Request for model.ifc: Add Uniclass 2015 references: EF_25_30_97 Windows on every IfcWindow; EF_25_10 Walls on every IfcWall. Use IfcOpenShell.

First a look at what the model holds.

```python
import ifcopenshell

model = ifcopenshell.open("model.ifc")
print(model.schema)
print("classifications:", [c.Name for c in model.by_type("IfcClassification")])
for ifc_class in ("IfcDoor", "IfcRoof", "IfcStair", "IfcWall", "IfcWindow"):
    print(ifc_class, len(model.by_type(ifc_class)))
```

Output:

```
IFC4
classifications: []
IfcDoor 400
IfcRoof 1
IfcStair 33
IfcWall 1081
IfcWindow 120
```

```python
import ifcopenshell
import ifcopenshell.api.classification

model = ifcopenshell.open("model.ifc")

system = ifcopenshell.api.classification.add_classification(model, classification="Uniclass 2015")

codes = {
    "IfcWindow": ("EF_25_30_97", "Windows"),
    "IfcWall": ("EF_25_10", "Walls"),
}
for ifc_class, (code, name) in codes.items():
    products = model.by_type(ifc_class)
    ifcopenshell.api.classification.add_reference(
        model, products=products, classification=system, identification=code, name=name
    )
    print(code, len(products))

model.write("model_updated.ifc")
```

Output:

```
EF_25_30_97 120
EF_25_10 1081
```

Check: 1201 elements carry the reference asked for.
